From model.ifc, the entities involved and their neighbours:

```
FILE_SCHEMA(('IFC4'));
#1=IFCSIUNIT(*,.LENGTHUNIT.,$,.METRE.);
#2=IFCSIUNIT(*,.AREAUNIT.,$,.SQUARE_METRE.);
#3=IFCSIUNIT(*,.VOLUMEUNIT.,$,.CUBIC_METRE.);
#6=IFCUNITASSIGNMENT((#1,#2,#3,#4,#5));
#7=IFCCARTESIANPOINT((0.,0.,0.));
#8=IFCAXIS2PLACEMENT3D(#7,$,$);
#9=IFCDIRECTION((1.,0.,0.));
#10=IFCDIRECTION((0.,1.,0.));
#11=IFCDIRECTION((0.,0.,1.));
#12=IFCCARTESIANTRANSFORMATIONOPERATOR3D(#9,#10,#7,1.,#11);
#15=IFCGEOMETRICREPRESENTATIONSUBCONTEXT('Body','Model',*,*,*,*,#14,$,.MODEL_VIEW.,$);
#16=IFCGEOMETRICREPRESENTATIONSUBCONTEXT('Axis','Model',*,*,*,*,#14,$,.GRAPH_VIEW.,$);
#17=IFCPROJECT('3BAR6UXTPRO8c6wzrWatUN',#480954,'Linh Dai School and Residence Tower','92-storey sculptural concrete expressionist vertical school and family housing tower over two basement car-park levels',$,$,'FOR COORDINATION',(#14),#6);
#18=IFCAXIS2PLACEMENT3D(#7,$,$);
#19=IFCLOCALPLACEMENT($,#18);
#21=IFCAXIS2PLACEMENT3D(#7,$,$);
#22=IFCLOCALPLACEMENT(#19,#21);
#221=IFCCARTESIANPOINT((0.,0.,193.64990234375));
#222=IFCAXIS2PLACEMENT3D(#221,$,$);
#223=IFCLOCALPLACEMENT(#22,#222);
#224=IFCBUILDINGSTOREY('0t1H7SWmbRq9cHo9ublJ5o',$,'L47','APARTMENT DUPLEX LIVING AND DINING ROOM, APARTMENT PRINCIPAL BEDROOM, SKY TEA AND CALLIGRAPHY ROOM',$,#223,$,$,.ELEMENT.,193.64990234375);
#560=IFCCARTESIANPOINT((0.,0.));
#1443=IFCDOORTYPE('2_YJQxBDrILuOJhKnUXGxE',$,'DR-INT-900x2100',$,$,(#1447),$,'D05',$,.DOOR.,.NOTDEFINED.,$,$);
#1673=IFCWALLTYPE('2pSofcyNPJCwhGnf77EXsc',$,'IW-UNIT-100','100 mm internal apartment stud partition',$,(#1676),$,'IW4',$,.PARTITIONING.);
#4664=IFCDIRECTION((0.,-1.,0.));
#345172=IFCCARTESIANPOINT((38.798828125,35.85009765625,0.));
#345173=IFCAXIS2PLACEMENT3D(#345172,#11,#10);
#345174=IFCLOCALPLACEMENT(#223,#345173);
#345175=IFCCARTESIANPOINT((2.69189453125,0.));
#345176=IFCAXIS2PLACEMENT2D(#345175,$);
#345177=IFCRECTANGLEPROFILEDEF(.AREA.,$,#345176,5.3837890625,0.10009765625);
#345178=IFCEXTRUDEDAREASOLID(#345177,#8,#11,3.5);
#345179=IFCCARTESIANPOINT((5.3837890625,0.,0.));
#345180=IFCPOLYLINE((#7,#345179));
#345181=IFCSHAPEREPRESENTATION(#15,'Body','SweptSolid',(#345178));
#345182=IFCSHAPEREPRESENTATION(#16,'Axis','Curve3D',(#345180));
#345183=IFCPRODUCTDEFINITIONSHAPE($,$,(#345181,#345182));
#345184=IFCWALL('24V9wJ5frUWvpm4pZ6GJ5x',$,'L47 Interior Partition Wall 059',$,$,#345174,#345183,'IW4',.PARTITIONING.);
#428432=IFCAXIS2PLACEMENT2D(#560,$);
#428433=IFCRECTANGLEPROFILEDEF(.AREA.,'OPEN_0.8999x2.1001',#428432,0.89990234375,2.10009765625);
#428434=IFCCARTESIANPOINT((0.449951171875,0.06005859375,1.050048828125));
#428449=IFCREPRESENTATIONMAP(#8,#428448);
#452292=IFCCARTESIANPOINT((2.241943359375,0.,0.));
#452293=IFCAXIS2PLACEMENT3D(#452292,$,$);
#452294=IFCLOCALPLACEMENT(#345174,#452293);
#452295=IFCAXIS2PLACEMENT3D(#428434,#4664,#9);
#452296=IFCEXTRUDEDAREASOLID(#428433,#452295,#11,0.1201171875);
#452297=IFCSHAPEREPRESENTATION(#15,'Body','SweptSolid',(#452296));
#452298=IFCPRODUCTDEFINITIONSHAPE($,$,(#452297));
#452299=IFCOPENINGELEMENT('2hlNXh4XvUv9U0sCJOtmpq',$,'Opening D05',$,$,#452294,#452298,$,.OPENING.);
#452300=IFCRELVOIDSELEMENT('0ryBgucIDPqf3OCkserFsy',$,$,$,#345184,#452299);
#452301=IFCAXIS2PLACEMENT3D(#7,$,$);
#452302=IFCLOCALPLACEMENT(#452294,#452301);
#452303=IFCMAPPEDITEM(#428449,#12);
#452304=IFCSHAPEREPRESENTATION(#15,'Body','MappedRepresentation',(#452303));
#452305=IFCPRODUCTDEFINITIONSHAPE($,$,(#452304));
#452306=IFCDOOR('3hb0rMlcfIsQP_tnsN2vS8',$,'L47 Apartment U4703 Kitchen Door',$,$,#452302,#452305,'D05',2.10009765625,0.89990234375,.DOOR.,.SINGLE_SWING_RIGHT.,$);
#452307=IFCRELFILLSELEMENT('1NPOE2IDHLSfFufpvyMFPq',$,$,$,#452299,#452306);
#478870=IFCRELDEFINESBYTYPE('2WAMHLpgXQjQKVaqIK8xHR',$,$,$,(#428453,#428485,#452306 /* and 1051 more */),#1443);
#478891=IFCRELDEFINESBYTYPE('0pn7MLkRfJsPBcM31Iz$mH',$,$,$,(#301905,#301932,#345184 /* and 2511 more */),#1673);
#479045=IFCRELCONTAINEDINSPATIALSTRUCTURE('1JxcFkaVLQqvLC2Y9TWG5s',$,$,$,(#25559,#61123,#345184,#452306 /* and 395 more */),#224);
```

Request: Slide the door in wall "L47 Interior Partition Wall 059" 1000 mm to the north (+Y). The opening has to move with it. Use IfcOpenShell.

```python
import ifcopenshell
import ifcopenshell.api.geometry
import ifcopenshell.util.placement

model = ifcopenshell.open("model.ifc")

door = model.by_guid("3hb0rMlcfIsQP_tnsN2vS8")
opening = door.FillsVoids[0].RelatingOpeningElement
wall = opening.VoidsElements[0].RelatingBuildingElement

wall_matrix = ifcopenshell.util.placement.get_local_placement(wall.ObjectPlacement)
shift = wall_matrix[:3, 0] * 1.0
before = ifcopenshell.util.placement.get_local_placement(door.ObjectPlacement)[:3, 3].copy()

# The door is placed relative to its opening, so it follows when the opening moves.
matrix = ifcopenshell.util.placement.get_local_placement(opening.ObjectPlacement)
matrix[:3, 3] += shift
ifcopenshell.api.geometry.edit_object_placement(
    model, product=opening, matrix=matrix, is_si=False, should_transform_children=True
)

after = ifcopenshell.util.placement.get_local_placement(door.ObjectPlacement)[:3, 3]
print("door moved by", (after - before).round(3) + 0.0)

model.write("model_edited.ifc")
```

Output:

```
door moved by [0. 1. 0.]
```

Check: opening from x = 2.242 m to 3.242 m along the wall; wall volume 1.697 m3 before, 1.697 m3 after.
